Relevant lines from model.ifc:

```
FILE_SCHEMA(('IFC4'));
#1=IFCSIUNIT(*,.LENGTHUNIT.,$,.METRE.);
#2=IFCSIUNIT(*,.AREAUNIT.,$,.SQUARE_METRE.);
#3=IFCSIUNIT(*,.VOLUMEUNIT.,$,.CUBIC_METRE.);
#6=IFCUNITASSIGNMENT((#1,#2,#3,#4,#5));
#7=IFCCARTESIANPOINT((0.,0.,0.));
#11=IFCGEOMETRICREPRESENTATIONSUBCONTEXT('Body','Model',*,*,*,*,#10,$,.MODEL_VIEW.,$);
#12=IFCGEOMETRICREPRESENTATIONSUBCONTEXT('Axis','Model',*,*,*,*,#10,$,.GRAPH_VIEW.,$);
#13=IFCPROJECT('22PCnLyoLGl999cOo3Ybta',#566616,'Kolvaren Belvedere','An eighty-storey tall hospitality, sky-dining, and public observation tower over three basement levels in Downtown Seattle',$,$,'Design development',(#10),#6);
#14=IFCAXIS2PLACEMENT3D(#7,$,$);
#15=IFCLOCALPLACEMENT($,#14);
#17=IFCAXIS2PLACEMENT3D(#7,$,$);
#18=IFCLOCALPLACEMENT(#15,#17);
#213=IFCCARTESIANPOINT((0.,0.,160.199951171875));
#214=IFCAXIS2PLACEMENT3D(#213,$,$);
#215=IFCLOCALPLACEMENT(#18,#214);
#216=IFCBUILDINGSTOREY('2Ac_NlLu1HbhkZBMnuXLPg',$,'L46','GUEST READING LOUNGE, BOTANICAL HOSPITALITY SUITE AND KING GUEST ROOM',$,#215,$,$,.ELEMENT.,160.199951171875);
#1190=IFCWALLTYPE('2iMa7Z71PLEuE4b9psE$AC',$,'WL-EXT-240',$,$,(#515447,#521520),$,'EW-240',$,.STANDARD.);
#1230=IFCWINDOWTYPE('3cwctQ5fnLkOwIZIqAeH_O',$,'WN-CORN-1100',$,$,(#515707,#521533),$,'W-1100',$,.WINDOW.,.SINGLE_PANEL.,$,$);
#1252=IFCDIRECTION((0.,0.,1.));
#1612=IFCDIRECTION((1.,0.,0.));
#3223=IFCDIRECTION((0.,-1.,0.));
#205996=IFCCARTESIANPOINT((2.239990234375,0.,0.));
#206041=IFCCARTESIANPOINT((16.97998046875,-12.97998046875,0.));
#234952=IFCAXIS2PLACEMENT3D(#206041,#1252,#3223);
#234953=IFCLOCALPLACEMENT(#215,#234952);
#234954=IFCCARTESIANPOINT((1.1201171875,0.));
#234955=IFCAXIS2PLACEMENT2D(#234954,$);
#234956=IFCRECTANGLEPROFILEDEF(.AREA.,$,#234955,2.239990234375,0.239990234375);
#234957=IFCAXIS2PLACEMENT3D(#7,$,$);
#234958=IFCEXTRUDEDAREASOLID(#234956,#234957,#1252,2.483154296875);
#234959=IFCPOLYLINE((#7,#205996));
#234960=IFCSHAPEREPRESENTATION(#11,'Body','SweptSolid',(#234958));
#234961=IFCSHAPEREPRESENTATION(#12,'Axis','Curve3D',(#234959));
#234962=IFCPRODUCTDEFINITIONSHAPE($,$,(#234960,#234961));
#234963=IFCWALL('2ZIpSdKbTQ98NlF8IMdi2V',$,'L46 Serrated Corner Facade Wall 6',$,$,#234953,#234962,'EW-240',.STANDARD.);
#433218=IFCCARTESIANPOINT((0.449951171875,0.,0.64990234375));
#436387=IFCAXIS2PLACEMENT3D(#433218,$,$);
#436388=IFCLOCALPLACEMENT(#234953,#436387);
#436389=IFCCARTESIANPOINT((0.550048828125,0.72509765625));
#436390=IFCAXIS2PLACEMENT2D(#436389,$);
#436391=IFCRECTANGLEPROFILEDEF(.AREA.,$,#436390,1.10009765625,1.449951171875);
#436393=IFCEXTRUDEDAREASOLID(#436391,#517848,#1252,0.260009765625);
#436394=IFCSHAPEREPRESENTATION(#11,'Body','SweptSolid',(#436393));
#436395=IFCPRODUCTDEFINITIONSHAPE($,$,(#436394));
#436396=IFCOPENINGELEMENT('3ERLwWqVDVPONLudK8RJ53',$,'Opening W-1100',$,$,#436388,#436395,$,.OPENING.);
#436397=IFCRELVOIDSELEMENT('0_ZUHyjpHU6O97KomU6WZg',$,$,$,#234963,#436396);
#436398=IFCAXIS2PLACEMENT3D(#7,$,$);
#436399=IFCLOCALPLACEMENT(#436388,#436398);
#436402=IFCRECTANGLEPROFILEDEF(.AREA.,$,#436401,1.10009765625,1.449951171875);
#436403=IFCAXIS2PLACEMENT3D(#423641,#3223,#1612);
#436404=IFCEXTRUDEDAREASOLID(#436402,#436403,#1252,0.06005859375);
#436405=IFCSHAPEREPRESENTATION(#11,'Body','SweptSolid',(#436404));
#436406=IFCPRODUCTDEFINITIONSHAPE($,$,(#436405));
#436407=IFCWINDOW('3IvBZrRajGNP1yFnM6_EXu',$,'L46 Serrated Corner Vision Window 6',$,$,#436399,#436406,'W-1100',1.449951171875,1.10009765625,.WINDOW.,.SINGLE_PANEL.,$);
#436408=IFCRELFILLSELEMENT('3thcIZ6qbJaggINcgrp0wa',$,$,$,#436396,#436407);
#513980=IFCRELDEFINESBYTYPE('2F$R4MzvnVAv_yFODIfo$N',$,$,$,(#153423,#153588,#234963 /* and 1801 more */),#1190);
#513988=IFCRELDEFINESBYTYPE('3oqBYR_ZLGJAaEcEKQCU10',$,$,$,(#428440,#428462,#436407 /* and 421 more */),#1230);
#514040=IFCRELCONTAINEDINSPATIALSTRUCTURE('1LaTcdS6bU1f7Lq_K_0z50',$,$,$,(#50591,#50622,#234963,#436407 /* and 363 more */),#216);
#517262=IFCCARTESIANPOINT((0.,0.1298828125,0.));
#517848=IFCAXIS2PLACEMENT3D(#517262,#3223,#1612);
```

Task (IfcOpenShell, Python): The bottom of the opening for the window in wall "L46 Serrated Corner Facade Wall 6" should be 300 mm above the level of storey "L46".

```python
import numpy as np
import ifcopenshell
import ifcopenshell.api.geometry
import ifcopenshell.geom
import ifcopenshell.util.element
import ifcopenshell.util.placement
import ifcopenshell.util.shape
import ifcopenshell.util.unit

model = ifcopenshell.open("model.ifc")
unit_scale = ifcopenshell.util.unit.calculate_unit_scale(model)

window = model.by_id(436407)
opening = window.FillsVoids[0].RelatingOpeningElement
storey = ifcopenshell.util.element.get_container(window, ifc_class="IfcBuildingStorey")
level = ifcopenshell.util.placement.get_local_placement(storey.ObjectPlacement)[2, 3]

# The opening's origin need not be at the sill, so measure its lowest point.
shape = ifcopenshell.geom.create_shape(ifcopenshell.geom.settings(), opening)
bottom = ifcopenshell.util.shape.get_shape_bottom_elevation(shape, shape.geometry) / unit_scale
dz = level + 0.3 / unit_scale - bottom

shift = np.array([0.0, 0.0, dz])
# The window is placed relative to its opening, so it follows when the opening moves.
matrix = ifcopenshell.util.placement.get_local_placement(opening.ObjectPlacement)
matrix[:3, 3] += shift
ifcopenshell.api.geometry.edit_object_placement(
    model, product=opening, matrix=matrix, is_si=False, should_transform_children=True
)

print(f"moved by {dz * unit_scale:+.3f} m")

model.write("model_updated.ifc")
```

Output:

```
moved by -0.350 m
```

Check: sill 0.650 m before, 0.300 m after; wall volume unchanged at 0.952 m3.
